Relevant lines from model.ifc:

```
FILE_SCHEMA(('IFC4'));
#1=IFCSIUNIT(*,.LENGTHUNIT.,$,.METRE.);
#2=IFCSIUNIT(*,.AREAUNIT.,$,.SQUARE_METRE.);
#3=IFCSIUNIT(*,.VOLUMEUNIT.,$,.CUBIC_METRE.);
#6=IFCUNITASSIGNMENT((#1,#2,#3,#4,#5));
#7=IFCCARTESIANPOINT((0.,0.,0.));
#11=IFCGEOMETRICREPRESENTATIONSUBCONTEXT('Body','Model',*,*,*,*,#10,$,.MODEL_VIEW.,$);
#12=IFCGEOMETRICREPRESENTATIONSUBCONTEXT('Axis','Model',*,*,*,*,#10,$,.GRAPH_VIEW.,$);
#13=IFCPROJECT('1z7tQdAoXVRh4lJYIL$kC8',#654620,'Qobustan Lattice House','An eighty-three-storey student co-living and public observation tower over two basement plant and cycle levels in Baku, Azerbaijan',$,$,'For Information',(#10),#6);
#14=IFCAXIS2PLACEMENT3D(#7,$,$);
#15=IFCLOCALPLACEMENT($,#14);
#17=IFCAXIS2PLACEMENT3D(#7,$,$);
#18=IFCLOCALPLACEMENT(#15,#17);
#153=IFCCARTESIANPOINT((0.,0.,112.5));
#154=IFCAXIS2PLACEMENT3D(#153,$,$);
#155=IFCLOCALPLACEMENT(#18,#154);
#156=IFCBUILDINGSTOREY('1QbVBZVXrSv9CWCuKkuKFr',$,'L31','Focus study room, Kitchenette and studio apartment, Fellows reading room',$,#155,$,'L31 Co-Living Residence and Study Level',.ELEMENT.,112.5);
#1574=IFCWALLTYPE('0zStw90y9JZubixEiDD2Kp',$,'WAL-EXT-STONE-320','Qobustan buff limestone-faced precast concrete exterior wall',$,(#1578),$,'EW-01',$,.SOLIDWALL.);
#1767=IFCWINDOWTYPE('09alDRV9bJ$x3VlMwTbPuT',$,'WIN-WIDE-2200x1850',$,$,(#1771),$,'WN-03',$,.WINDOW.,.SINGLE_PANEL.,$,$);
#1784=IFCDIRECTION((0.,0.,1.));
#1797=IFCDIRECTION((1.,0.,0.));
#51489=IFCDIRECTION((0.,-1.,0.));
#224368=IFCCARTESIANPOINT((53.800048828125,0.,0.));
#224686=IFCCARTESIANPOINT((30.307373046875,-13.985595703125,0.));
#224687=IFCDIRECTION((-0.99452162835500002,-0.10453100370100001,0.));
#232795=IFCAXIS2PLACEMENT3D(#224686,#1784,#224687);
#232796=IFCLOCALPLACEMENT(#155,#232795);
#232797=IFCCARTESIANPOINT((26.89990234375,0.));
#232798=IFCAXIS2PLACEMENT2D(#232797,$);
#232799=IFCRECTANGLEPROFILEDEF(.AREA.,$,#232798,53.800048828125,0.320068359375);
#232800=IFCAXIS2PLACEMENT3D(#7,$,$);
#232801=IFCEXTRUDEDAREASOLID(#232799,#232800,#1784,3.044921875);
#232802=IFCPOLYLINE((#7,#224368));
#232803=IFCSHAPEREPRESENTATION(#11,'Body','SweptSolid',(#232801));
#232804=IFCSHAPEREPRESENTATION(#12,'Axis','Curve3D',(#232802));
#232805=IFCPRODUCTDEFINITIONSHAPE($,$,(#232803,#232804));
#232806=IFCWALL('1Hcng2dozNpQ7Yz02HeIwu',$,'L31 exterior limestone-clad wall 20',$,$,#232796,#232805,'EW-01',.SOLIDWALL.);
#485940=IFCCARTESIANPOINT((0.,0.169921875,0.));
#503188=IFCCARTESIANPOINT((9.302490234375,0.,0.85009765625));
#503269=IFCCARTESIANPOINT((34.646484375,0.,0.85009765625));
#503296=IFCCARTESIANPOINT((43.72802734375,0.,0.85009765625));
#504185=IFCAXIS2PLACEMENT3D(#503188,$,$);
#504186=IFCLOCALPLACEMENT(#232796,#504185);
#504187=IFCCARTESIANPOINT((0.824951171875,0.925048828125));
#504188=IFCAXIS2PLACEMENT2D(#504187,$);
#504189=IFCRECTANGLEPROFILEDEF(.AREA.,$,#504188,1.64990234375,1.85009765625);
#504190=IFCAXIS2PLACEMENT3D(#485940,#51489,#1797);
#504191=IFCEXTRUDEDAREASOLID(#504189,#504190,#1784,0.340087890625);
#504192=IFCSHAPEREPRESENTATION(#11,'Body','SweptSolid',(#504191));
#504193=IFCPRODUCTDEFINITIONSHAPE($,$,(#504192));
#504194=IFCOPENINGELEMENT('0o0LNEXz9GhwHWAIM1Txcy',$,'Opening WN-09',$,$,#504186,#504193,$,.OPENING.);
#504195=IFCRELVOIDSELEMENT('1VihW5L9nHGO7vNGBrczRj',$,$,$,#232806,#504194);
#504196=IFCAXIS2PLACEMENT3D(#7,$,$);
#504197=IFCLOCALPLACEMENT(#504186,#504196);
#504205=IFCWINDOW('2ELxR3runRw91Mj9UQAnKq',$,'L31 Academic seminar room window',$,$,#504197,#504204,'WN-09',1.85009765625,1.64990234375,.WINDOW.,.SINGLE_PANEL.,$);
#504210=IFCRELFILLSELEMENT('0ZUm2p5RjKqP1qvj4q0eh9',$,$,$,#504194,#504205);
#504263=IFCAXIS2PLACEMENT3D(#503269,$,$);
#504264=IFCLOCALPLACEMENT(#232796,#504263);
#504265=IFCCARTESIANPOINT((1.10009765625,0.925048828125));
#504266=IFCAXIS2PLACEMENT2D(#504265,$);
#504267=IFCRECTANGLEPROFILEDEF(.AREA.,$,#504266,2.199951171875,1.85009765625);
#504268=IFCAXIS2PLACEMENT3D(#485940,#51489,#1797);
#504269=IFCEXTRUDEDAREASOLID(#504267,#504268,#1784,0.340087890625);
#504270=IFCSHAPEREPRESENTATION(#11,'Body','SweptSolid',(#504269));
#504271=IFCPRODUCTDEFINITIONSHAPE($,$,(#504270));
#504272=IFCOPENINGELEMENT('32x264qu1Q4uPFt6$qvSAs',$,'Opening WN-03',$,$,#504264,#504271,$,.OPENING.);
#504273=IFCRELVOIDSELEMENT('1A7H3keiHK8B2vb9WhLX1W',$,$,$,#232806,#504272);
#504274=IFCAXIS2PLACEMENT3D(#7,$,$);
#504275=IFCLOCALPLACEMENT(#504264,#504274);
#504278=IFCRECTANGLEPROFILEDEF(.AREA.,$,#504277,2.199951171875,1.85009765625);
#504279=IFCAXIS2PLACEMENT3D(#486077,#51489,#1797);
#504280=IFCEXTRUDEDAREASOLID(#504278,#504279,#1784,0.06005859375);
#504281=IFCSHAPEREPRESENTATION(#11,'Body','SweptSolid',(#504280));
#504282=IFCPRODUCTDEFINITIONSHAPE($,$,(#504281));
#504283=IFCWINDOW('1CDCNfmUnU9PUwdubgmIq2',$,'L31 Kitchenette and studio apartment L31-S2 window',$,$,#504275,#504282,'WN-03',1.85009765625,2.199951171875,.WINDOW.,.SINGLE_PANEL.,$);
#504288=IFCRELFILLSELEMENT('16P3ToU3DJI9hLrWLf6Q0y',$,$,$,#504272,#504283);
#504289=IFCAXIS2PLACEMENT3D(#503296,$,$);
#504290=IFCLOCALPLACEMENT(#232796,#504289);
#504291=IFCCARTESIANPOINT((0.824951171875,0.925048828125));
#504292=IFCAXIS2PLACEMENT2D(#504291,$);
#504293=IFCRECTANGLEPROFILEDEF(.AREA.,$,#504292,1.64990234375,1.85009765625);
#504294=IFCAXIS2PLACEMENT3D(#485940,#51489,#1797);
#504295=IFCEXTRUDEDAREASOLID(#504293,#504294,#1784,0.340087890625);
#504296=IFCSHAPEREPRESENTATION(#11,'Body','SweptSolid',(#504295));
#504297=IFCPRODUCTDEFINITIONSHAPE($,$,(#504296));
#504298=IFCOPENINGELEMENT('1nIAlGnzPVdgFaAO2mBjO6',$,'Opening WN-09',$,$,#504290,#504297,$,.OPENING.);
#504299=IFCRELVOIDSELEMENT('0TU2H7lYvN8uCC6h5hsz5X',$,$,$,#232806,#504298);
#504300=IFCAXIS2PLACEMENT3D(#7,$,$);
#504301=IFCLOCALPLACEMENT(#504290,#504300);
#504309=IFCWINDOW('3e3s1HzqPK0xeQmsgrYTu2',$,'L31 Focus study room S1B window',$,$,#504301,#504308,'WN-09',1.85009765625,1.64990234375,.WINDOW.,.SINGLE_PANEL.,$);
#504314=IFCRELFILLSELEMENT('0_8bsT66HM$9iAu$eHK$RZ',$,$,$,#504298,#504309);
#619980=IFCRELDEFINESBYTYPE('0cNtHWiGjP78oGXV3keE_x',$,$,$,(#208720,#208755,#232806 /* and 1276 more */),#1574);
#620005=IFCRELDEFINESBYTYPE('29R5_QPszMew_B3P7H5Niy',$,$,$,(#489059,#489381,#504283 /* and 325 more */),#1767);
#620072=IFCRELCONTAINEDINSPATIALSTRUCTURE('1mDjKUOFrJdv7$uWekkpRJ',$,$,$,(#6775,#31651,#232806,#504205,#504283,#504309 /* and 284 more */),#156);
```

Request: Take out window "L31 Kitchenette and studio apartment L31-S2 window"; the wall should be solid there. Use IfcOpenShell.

```python
import ifcopenshell
import ifcopenshell.api.feature
import ifcopenshell.api.root
import ifcopenshell.geom
import ifcopenshell.util.shape

model = ifcopenshell.open("model.ifc")
settings = ifcopenshell.geom.settings()


def volume(element):
    """Net volume in cubic metres, openings subtracted."""
    shape = ifcopenshell.geom.create_shape(settings, element)
    return ifcopenshell.util.shape.get_volume(shape.geometry)


window = model.by_guid("1CDCNfmUnU9PUwdubgmIq2")
opening = window.FillsVoids[0].RelatingOpeningElement
wall = opening.VoidsElements[0].RelatingBuildingElement
before = volume(wall)

ifcopenshell.api.root.remove_product(model, product=window)
ifcopenshell.api.feature.remove_feature(model, feature=opening)

after = volume(wall)

print(f"wall volume {before:.3f} -> {after:.3f} m3")

model.write("model_v2.ifc")
```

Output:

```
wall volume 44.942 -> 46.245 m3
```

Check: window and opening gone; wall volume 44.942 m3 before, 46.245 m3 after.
